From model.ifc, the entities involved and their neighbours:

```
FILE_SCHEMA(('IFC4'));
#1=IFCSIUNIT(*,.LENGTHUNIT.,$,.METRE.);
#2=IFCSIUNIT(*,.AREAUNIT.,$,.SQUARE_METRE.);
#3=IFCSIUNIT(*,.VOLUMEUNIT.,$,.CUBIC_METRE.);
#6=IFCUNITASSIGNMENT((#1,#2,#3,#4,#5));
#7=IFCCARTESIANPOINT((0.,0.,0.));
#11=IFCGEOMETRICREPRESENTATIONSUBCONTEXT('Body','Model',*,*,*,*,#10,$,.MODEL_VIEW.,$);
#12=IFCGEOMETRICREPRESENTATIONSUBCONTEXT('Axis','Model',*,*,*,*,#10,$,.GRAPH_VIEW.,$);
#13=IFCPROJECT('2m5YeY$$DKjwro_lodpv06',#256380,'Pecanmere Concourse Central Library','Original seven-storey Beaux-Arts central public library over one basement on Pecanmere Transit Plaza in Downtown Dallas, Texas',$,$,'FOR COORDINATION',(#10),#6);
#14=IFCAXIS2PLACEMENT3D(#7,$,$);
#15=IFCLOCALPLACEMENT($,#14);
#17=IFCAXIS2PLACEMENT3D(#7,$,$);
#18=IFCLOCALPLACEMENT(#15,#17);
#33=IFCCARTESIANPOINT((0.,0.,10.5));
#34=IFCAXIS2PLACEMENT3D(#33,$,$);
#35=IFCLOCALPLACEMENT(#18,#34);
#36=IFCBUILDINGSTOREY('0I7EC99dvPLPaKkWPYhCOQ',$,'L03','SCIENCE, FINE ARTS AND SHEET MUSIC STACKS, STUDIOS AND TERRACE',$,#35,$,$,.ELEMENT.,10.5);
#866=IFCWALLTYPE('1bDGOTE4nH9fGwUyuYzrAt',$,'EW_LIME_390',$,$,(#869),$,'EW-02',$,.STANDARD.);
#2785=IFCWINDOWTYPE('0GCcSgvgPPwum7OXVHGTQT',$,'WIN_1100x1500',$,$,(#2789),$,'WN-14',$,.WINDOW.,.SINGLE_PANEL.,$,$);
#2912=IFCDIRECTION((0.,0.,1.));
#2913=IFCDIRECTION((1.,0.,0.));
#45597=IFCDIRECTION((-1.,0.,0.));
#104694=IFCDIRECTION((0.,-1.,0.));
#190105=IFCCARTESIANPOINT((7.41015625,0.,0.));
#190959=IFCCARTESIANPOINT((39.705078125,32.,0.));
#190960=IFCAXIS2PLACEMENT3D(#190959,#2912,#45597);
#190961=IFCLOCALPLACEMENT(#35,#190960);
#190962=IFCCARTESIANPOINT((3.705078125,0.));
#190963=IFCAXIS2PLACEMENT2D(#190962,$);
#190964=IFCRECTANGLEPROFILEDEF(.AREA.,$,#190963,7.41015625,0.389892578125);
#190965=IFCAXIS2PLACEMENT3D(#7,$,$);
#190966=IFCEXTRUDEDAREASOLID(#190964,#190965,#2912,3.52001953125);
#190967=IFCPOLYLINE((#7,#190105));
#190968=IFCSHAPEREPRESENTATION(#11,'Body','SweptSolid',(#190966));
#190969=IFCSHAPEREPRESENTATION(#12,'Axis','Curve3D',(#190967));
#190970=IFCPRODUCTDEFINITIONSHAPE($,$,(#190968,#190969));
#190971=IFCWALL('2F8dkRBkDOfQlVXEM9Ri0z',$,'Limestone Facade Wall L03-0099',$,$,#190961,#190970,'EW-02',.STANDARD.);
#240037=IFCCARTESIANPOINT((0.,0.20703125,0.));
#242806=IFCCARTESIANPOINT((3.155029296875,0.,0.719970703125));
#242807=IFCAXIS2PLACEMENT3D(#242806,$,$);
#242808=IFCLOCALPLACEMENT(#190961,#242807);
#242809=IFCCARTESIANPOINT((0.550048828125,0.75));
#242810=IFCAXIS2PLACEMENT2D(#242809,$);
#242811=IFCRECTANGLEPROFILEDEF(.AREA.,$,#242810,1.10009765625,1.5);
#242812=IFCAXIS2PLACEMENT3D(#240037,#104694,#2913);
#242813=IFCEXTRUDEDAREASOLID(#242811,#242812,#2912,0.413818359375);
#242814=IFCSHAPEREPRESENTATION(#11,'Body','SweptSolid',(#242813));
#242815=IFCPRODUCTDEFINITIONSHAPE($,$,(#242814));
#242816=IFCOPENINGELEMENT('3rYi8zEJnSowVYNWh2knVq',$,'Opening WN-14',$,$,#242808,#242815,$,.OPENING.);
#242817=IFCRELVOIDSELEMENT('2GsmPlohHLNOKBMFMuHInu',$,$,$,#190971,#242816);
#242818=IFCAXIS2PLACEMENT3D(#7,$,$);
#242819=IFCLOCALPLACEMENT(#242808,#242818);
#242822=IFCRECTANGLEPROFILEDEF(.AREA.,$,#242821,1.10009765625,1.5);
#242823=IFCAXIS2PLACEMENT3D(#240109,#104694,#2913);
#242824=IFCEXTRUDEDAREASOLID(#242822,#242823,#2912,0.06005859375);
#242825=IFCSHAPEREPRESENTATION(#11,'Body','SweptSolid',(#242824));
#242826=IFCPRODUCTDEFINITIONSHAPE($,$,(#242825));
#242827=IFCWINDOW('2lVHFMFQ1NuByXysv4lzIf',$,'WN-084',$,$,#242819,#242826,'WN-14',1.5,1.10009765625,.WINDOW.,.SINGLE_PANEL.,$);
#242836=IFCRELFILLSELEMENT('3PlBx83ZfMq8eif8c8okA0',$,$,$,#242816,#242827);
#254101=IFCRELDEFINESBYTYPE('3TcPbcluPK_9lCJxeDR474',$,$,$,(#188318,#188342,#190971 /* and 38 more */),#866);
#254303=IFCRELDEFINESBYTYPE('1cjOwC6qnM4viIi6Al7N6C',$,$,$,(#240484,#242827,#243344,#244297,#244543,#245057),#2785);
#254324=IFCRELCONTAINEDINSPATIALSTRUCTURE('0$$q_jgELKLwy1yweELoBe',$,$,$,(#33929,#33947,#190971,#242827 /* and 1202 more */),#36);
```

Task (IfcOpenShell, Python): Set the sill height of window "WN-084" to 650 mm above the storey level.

```python
import numpy as np
import ifcopenshell
import ifcopenshell.api.geometry
import ifcopenshell.geom
import ifcopenshell.util.element
import ifcopenshell.util.placement
import ifcopenshell.util.shape
import ifcopenshell.util.unit

model = ifcopenshell.open("model.ifc")
unit_scale = ifcopenshell.util.unit.calculate_unit_scale(model)

window = model.by_guid("2lVHFMFQ1NuByXysv4lzIf")
opening = window.FillsVoids[0].RelatingOpeningElement
storey = ifcopenshell.util.element.get_container(window, ifc_class="IfcBuildingStorey")
level = ifcopenshell.util.placement.get_local_placement(storey.ObjectPlacement)[2, 3]

# The opening's origin need not be at the sill, so measure its lowest point.
shape = ifcopenshell.geom.create_shape(ifcopenshell.geom.settings(), opening)
bottom = ifcopenshell.util.shape.get_shape_bottom_elevation(shape, shape.geometry) / unit_scale
dz = level + 0.65 - bottom

shift = np.array([0.0, 0.0, dz])
# The window is placed relative to its opening, so it follows when the opening moves.
matrix = ifcopenshell.util.placement.get_local_placement(opening.ObjectPlacement)
matrix[:3, 3] += shift
ifcopenshell.api.geometry.edit_object_placement(
    model, product=opening, matrix=matrix, is_si=False, should_transform_children=True
)

print(f"moved by {dz * unit_scale:+.3f} m")

model.write("model_v2.ifc")
```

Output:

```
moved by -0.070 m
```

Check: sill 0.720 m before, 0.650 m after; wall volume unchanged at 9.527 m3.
